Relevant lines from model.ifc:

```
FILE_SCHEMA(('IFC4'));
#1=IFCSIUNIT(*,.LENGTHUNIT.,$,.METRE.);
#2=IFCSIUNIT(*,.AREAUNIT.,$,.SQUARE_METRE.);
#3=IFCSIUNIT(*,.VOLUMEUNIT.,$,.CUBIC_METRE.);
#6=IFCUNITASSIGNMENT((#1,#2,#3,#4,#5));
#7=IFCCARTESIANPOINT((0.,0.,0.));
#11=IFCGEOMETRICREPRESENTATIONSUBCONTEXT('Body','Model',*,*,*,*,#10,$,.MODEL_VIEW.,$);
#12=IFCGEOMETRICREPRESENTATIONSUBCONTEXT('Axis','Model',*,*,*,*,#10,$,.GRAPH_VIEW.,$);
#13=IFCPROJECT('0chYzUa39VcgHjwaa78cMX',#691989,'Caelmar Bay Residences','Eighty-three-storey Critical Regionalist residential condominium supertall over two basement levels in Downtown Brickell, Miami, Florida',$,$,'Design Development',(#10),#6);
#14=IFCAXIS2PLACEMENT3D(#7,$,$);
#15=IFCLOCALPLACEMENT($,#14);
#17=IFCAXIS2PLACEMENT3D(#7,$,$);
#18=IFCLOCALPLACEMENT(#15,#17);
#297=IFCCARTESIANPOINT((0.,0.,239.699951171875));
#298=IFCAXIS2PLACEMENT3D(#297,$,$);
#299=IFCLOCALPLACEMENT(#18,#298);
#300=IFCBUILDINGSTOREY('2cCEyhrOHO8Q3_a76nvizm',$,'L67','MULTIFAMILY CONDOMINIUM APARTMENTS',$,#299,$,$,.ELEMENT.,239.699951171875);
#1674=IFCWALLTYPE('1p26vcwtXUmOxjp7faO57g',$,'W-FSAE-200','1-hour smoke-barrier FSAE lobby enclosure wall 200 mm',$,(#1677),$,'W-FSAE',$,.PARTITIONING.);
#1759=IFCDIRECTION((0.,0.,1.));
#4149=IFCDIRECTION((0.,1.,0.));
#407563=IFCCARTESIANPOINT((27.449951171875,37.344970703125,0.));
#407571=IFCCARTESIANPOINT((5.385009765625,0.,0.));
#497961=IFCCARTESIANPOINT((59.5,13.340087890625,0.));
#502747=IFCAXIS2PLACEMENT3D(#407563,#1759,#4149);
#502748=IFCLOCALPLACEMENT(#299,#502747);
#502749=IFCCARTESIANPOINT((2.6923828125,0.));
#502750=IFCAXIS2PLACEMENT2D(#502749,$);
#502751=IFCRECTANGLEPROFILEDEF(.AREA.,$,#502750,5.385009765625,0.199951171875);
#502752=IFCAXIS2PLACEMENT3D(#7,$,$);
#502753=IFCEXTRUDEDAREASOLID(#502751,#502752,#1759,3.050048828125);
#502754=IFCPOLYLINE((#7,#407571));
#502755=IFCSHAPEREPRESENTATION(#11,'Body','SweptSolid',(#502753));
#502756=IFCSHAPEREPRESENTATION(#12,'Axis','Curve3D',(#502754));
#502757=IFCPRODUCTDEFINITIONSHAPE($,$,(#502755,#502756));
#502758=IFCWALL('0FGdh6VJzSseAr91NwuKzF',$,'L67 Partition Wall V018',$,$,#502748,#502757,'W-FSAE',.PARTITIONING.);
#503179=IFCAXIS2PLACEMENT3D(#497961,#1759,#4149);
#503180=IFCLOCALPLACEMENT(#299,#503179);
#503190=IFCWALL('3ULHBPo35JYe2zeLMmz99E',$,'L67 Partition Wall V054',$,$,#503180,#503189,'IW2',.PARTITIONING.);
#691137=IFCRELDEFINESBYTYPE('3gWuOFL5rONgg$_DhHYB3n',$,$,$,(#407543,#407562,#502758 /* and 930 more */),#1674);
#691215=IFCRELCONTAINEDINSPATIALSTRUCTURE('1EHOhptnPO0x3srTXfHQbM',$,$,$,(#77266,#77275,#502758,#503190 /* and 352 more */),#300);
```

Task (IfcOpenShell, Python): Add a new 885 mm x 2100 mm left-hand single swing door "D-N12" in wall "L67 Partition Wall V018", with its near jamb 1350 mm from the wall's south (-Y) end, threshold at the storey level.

```python
import numpy as np
import ifcopenshell
import ifcopenshell.api.feature
import ifcopenshell.api.geometry
import ifcopenshell.api.root
import ifcopenshell.api.spatial
import ifcopenshell.geom
import ifcopenshell.util.element
import ifcopenshell.util.placement
import ifcopenshell.util.representation
import ifcopenshell.util.shape
import ifcopenshell.util.unit

model = ifcopenshell.open("model.ifc")
unit_scale = ifcopenshell.util.unit.calculate_unit_scale(model)
settings = ifcopenshell.geom.settings()


def volume(element):
    """Net volume in cubic metres, openings subtracted."""
    shape = ifcopenshell.geom.create_shape(settings, element)
    return ifcopenshell.util.shape.get_volume(shape.geometry)


wall = model.by_guid("0FGdh6VJzSseAr91NwuKzF")
storey = ifcopenshell.util.element.get_container(wall, ifc_class="IfcBuildingStorey")
context = ifcopenshell.util.representation.get_context(model, "Model", "Body", "MODEL_VIEW")
before = volume(wall)

width, height, from_end, sill = 0.885, 2.1, 1.35, 0.0  # metres

# The wall runs along its own X axis, and the end named is its -X end.
wall_shape = ifcopenshell.geom.create_shape(settings, wall)
x, y, z = ifcopenshell.util.shape.get_vertices(wall_shape.geometry).T
start = x.min() + from_end
face, thickness = float(y.min()), float(y.max() - y.min())
wall_matrix = ifcopenshell.util.placement.get_local_placement(wall.ObjectPlacement)
level = ifcopenshell.util.placement.get_local_placement(storey.ObjectPlacement)[2, 3]


def in_wall(x, y):
    """Placement at x, y metres in the wall's axes, at sill height."""
    matrix = wall_matrix.copy()
    matrix[:, 3] = wall_matrix @ np.array([x / unit_scale, y / unit_scale, 0.0, 1.0])
    matrix[2, 3] = level + sill / unit_scale
    return matrix


# Opening: a box that overshoots both wall faces by 50 mm.
opening = ifcopenshell.api.root.create_entity(model, ifc_class="IfcOpeningElement", predefined_type="OPENING")
box = ifcopenshell.api.geometry.add_wall_representation(
    model, context=context, length=width, height=height, thickness=thickness + 0.1
)
ifcopenshell.api.geometry.assign_representation(model, product=opening, representation=box)
ifcopenshell.api.geometry.edit_object_placement(model, product=opening, matrix=in_wall(start, face - 0.05), is_si=False)
ifcopenshell.api.feature.add_feature(model, feature=opening, element=wall)

door = ifcopenshell.api.root.create_entity(model, ifc_class="IfcDoor", name="D-N12", predefined_type="DOOR")
door.OverallWidth, door.OverallHeight = width / unit_scale, height / unit_scale
door.OperationType = "SINGLE_SWING_LEFT"
body = ifcopenshell.api.geometry.add_door_representation(
    model,
    context=context,
    overall_width=door.OverallWidth,
    overall_height=door.OverallHeight,
    operation_type="SINGLE_SWING_LEFT",
    lining_properties={"LiningDepth": thickness / unit_scale, "ThresholdDepth": thickness / unit_scale},
)
ifcopenshell.api.geometry.assign_representation(model, product=door, representation=body)
ifcopenshell.api.spatial.assign_container(model, products=[door], relating_structure=storey)
ifcopenshell.api.feature.add_filling(model, opening=opening, element=door)

# The lining spans the wall, so the door starts at the wall face.
ifcopenshell.api.geometry.edit_object_placement(model, product=door, matrix=in_wall(start, face), is_si=False)

after = volume(wall)

print(f"wall volume {before:.3f} -> {after:.3f} m3")

model.write("model-out.ifc")
```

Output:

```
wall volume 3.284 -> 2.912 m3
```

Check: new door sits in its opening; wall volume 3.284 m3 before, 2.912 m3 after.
